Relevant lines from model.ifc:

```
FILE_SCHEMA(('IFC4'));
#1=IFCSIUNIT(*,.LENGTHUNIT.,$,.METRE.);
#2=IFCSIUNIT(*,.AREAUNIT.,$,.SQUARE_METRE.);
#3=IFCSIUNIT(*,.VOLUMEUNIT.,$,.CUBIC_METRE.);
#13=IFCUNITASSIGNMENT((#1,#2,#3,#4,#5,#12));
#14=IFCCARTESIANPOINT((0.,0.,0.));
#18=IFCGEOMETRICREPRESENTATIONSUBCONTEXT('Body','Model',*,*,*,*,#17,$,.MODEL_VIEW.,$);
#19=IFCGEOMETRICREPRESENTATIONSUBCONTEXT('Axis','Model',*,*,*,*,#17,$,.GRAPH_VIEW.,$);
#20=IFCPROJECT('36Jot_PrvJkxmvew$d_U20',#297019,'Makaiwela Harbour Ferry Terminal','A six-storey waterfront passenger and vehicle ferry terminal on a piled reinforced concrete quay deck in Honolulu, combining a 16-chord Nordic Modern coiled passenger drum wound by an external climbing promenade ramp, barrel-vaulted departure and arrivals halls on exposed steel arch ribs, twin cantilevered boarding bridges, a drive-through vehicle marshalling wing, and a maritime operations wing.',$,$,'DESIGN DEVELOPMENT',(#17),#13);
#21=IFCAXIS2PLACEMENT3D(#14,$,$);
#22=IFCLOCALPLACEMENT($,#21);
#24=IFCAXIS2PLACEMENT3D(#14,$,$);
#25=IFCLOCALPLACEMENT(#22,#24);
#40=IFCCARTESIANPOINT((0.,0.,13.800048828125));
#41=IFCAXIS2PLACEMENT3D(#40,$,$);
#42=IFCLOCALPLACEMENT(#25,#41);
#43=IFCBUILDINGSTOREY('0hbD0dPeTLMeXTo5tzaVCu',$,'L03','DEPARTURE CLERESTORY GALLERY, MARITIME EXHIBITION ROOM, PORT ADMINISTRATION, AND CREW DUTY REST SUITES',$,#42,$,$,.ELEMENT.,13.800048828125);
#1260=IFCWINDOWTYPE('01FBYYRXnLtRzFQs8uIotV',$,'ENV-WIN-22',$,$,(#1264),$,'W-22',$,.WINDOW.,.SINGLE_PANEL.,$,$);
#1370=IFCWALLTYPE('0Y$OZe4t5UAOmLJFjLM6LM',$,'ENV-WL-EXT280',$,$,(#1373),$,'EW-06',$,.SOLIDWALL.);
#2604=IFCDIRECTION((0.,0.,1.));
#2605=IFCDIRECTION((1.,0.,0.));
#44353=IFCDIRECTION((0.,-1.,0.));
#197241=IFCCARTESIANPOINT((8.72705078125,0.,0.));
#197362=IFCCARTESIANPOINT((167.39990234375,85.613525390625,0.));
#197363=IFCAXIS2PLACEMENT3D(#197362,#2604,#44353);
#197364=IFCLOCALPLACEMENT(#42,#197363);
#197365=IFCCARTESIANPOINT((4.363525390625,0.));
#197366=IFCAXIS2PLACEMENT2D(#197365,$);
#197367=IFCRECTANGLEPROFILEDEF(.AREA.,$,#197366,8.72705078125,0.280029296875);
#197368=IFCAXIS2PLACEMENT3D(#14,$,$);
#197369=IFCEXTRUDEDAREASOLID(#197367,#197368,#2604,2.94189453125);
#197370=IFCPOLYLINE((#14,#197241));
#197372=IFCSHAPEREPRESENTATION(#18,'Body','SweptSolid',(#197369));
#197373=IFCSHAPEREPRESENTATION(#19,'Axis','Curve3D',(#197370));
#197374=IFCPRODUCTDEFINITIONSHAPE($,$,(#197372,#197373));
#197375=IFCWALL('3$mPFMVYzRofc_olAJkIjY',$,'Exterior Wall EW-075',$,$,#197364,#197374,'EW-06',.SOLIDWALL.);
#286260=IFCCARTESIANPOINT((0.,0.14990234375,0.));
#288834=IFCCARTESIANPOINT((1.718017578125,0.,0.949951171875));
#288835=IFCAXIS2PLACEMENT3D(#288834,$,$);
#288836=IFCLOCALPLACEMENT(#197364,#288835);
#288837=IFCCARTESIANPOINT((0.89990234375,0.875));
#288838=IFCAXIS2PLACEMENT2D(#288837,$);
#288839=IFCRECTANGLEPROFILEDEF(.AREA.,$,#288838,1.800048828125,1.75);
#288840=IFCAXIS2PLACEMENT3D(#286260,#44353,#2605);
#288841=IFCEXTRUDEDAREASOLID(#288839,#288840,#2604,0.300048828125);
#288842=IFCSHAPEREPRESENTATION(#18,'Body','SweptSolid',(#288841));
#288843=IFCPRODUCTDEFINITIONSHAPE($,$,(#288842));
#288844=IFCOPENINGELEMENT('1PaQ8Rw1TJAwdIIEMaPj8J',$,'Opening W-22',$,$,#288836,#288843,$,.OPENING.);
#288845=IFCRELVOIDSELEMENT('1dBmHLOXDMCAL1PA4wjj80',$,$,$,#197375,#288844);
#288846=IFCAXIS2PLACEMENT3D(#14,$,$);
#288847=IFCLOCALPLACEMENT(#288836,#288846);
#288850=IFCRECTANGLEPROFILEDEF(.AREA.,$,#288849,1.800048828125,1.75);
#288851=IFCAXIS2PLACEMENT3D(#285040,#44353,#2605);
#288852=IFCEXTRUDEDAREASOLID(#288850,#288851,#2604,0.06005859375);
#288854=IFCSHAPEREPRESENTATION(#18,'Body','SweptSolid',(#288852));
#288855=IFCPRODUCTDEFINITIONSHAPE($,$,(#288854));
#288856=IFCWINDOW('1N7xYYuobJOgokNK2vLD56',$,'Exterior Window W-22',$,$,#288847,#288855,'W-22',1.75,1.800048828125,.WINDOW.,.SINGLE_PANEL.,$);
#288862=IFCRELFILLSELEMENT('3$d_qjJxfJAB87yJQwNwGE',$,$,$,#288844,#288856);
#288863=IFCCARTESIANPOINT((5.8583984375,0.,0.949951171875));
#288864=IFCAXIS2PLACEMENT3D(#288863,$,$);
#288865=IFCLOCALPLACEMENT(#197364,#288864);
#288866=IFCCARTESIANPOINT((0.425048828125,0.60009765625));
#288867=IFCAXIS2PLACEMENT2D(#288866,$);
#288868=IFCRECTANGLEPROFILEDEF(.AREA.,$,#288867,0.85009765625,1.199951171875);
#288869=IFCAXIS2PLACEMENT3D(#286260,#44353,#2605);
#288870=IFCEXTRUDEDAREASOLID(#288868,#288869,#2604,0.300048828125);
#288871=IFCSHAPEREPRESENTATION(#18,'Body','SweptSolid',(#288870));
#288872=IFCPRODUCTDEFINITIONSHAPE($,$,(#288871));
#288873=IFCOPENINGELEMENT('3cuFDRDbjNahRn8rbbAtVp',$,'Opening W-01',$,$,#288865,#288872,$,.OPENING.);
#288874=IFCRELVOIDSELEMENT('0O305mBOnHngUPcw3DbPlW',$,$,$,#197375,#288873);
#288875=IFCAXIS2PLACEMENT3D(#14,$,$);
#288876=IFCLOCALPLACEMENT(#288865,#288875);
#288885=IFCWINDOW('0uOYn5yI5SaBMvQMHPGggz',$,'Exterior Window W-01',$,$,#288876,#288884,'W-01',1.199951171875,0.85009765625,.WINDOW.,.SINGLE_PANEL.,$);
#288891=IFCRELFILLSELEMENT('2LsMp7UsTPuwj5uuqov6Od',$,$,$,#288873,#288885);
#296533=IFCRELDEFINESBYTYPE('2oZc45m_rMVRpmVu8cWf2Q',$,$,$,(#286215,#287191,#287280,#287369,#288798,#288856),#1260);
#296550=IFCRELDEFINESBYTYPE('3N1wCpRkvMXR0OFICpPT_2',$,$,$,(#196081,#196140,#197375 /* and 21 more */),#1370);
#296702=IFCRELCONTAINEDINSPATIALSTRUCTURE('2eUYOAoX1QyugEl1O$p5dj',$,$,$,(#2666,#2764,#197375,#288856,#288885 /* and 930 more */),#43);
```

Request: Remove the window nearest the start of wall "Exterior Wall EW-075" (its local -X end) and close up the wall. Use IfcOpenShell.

```python
import ifcopenshell
import ifcopenshell.api.feature
import ifcopenshell.api.root
import ifcopenshell.geom
import ifcopenshell.util.shape

model = ifcopenshell.open("model.ifc")
settings = ifcopenshell.geom.settings()


def volume(element):
    """Net volume in cubic metres, openings subtracted."""
    shape = ifcopenshell.geom.create_shape(settings, element)
    return ifcopenshell.util.shape.get_volume(shape.geometry)


window = model.by_id(288856)
opening = window.FillsVoids[0].RelatingOpeningElement
wall = opening.VoidsElements[0].RelatingBuildingElement
before = volume(wall)

ifcopenshell.api.root.remove_product(model, product=window)
ifcopenshell.api.feature.remove_feature(model, feature=opening)

after = volume(wall)

print(f"wall volume {before:.3f} -> {after:.3f} m3")

model.write("model_updated.ifc")
```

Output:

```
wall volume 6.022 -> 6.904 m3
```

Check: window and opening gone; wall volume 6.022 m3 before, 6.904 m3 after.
